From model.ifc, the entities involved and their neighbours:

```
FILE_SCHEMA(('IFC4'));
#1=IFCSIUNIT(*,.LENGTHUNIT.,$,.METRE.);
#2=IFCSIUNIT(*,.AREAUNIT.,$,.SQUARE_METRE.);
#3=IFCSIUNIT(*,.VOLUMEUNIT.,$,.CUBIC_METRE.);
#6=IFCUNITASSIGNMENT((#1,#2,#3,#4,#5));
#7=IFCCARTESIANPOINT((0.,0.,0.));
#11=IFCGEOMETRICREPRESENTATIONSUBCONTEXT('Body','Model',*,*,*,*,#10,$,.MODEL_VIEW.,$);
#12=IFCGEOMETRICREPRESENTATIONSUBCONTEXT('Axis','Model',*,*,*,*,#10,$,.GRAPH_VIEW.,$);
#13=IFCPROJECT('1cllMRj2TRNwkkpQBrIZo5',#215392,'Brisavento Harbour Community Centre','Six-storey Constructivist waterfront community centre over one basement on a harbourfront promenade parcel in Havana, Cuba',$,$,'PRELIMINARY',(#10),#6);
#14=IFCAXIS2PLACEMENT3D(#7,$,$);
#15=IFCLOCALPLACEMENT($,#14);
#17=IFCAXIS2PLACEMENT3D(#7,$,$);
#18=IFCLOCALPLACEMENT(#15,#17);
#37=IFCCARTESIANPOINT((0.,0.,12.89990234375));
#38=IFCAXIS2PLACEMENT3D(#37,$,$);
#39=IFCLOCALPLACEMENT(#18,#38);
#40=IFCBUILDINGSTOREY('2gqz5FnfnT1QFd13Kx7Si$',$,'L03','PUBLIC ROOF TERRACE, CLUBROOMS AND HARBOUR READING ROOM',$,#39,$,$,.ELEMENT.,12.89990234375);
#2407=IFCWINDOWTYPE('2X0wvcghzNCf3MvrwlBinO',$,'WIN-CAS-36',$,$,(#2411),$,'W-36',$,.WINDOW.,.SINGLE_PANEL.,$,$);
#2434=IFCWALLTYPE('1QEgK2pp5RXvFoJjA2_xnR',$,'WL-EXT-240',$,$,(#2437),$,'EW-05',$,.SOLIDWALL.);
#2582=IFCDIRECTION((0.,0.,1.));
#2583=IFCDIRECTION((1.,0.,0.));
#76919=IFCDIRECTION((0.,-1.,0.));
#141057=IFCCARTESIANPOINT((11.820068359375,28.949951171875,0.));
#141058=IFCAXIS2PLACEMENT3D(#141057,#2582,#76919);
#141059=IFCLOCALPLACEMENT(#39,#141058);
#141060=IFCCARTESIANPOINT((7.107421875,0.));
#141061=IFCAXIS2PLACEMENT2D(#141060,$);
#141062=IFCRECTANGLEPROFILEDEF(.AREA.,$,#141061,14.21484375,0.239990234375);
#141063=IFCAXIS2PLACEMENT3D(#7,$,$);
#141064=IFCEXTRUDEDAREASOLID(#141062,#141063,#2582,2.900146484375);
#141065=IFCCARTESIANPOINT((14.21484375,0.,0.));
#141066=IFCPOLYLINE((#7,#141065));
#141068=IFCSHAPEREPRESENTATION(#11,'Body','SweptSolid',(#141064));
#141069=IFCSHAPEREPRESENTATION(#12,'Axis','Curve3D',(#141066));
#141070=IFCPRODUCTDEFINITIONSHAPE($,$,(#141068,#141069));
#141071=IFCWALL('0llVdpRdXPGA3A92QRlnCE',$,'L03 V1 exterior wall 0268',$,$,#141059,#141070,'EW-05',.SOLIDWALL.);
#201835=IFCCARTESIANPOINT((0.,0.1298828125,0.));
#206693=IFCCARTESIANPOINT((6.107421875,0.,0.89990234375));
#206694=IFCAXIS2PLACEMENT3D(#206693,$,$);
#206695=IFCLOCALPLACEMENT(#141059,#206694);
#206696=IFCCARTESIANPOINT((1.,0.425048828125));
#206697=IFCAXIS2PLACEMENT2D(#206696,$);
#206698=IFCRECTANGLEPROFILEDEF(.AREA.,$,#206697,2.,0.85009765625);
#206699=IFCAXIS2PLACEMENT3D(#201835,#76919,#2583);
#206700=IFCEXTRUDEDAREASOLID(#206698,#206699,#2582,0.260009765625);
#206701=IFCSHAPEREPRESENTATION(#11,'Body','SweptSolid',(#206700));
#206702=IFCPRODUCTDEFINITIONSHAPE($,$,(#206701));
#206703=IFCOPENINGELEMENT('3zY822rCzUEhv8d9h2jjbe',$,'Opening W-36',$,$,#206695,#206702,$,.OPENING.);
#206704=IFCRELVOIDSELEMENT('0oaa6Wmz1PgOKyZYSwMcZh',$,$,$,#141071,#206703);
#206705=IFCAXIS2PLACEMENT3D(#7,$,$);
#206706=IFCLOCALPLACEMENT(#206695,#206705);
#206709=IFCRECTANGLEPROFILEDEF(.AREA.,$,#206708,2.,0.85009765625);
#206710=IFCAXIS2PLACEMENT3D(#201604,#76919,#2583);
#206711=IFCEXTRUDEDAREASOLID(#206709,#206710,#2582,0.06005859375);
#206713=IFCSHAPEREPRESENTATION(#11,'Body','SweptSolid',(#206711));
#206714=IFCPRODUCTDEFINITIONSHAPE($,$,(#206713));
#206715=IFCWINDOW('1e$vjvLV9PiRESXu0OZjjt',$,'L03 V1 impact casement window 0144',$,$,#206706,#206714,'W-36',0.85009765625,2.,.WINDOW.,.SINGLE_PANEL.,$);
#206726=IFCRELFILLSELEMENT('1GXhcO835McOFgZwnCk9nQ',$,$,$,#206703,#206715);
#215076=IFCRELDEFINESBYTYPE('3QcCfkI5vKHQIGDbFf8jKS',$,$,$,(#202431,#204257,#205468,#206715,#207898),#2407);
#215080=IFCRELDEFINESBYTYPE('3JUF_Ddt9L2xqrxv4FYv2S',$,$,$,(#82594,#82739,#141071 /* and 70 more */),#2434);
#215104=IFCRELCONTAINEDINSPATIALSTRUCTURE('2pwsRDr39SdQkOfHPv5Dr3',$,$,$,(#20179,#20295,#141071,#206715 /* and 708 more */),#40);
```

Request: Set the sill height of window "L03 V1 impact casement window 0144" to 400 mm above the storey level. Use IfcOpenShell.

```python
import numpy as np
import ifcopenshell
import ifcopenshell.api.geometry
import ifcopenshell.geom
import ifcopenshell.util.element
import ifcopenshell.util.placement
import ifcopenshell.util.shape
import ifcopenshell.util.unit

model = ifcopenshell.open("model.ifc")
unit_scale = ifcopenshell.util.unit.calculate_unit_scale(model)

window = model.by_id(206715)
opening = window.FillsVoids[0].RelatingOpeningElement
storey = ifcopenshell.util.element.get_container(window, ifc_class="IfcBuildingStorey")
level = ifcopenshell.util.placement.get_local_placement(storey.ObjectPlacement)[2, 3]

# The opening's origin need not be at the sill, so measure its lowest point.
shape = ifcopenshell.geom.create_shape(ifcopenshell.geom.settings(), opening)
bottom = ifcopenshell.util.shape.get_shape_bottom_elevation(shape, shape.geometry) / unit_scale
dz = level + 0.4 / unit_scale - bottom

shift = np.array([0.0, 0.0, dz])
# The window is placed relative to its opening, so it follows when the opening moves.
matrix = ifcopenshell.util.placement.get_local_placement(opening.ObjectPlacement)
matrix[:3, 3] += shift
ifcopenshell.api.geometry.edit_object_placement(
    model, product=opening, matrix=matrix, is_si=False, should_transform_children=True
)

print(f"moved by {dz * unit_scale:+.3f} m")

model.write("model_edited.ifc")
```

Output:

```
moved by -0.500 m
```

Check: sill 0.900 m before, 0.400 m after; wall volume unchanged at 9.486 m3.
